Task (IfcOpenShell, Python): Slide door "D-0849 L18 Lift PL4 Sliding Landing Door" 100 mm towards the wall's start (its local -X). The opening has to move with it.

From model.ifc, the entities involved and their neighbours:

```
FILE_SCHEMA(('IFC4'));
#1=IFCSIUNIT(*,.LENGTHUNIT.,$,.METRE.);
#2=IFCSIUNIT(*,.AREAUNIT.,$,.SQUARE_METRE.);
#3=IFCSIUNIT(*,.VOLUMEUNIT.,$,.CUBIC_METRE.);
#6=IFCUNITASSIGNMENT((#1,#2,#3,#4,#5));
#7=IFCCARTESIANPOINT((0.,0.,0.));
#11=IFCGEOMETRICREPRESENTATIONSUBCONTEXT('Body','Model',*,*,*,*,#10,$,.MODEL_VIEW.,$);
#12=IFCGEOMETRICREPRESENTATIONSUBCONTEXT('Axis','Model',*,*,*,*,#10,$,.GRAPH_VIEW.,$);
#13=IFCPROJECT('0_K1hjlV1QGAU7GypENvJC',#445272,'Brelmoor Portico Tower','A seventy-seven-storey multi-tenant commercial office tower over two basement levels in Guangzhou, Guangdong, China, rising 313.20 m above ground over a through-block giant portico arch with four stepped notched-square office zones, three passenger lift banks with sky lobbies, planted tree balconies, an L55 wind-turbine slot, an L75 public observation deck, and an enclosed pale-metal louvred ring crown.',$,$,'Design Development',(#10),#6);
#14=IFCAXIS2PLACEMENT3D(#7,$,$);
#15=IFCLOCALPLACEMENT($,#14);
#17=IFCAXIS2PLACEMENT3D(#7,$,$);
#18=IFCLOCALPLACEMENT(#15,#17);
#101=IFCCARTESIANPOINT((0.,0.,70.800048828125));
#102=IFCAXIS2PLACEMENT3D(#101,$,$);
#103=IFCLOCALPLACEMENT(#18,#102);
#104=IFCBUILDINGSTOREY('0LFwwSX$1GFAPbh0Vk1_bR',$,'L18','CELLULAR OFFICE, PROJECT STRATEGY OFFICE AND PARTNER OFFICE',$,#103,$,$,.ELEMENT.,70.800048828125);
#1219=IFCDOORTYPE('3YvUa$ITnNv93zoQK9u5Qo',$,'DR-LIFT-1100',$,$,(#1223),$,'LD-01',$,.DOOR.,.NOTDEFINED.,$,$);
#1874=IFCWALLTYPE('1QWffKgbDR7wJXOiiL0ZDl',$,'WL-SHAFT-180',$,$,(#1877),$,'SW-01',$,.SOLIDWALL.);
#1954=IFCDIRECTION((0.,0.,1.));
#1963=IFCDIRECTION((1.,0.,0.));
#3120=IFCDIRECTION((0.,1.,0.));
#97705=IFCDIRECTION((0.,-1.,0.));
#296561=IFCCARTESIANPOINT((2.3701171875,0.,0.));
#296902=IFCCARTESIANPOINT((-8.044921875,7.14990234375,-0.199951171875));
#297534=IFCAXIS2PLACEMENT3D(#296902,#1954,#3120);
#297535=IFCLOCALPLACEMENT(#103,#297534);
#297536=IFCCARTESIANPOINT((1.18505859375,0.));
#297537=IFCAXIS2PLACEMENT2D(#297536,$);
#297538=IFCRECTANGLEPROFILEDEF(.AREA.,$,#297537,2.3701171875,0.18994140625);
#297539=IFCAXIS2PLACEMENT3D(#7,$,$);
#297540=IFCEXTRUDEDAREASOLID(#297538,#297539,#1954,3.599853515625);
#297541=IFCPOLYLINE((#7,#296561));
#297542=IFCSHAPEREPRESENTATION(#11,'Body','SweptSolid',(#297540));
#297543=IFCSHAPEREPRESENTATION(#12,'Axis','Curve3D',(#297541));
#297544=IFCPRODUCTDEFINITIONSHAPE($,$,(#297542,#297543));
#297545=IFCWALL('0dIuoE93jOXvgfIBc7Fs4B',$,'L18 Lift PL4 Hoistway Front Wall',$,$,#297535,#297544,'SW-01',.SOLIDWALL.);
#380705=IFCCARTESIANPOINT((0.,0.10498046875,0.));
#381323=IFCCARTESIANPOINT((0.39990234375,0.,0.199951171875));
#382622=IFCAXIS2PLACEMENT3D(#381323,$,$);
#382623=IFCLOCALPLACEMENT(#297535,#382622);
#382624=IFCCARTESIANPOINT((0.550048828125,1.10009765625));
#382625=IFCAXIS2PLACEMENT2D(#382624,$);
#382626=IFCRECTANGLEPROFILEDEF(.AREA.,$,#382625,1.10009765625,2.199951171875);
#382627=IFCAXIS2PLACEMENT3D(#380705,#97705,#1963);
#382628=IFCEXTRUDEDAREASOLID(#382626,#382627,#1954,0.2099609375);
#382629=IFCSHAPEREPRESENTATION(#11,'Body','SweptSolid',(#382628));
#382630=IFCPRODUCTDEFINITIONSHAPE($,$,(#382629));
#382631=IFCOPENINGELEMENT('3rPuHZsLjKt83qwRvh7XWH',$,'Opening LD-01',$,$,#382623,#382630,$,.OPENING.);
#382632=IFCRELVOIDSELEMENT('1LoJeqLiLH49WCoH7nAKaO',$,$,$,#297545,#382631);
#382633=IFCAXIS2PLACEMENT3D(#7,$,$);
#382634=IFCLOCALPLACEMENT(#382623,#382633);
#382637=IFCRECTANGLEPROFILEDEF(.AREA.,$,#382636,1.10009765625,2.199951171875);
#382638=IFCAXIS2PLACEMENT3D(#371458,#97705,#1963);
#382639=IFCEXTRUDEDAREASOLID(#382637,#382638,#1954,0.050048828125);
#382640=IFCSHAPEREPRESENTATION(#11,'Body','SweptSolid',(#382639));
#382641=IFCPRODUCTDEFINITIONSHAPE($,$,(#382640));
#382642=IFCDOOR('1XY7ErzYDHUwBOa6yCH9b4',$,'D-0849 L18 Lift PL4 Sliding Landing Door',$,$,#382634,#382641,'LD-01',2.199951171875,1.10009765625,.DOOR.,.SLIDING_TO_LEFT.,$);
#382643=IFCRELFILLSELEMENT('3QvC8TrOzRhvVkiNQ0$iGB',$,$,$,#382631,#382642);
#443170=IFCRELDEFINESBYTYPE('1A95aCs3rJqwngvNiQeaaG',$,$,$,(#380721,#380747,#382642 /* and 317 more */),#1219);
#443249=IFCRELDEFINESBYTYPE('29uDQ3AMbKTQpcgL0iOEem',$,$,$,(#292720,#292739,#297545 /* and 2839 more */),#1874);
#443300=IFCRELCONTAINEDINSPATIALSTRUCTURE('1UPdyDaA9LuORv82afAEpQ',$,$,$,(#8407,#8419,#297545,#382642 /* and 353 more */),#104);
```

```python
import ifcopenshell
import ifcopenshell.api.geometry
import ifcopenshell.util.placement
import ifcopenshell.util.unit

model = ifcopenshell.open("model.ifc")
unit_scale = ifcopenshell.util.unit.calculate_unit_scale(model)

door = model.by_guid("1XY7ErzYDHUwBOa6yCH9b4")
opening = door.FillsVoids[0].RelatingOpeningElement
wall = opening.VoidsElements[0].RelatingBuildingElement

wall_matrix = ifcopenshell.util.placement.get_local_placement(wall.ObjectPlacement)
shift = wall_matrix[:3, 0] * -0.1 / unit_scale
before = ifcopenshell.util.placement.get_local_placement(door.ObjectPlacement)[:3, 3].copy()

# The door is placed relative to its opening, so it follows when the opening moves.
matrix = ifcopenshell.util.placement.get_local_placement(opening.ObjectPlacement)
matrix[:3, 3] += shift
ifcopenshell.api.geometry.edit_object_placement(
    model, product=opening, matrix=matrix, is_si=False, should_transform_children=True
)

after = ifcopenshell.util.placement.get_local_placement(door.ObjectPlacement)[:3, 3]
print("door moved by", (after - before).round(3) + 0.0)

model.write("model_v2.ifc")
```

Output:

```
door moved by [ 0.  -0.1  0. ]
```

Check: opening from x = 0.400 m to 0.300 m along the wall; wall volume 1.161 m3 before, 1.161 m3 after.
